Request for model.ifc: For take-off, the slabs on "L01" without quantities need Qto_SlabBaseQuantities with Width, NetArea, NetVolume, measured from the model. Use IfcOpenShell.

First a look at what the model holds.

```python
import ifcopenshell
import ifcopenshell.util.element
import ifcopenshell.util.unit

model = ifcopenshell.open("model.ifc")
print(model.schema)
for unit_type in ("LENGTHUNIT", "AREAUNIT", "VOLUMEUNIT"):
    print(unit_type, ifcopenshell.util.unit.calculate_unit_scale(model, unit_type))
storey = next(s for s in model.by_type("IfcBuildingStorey") if s.Name == "L01")
slabs = [e for e in ifcopenshell.util.element.get_decomposition(storey) if e.is_a("IfcSlab")]
for e in sorted(slabs, key=lambda e: e.id()):
    print(e.id(), e.is_a(), e.Name, list(ifcopenshell.util.element.get_psets(e, qtos_only=True)), sep=" | ")
```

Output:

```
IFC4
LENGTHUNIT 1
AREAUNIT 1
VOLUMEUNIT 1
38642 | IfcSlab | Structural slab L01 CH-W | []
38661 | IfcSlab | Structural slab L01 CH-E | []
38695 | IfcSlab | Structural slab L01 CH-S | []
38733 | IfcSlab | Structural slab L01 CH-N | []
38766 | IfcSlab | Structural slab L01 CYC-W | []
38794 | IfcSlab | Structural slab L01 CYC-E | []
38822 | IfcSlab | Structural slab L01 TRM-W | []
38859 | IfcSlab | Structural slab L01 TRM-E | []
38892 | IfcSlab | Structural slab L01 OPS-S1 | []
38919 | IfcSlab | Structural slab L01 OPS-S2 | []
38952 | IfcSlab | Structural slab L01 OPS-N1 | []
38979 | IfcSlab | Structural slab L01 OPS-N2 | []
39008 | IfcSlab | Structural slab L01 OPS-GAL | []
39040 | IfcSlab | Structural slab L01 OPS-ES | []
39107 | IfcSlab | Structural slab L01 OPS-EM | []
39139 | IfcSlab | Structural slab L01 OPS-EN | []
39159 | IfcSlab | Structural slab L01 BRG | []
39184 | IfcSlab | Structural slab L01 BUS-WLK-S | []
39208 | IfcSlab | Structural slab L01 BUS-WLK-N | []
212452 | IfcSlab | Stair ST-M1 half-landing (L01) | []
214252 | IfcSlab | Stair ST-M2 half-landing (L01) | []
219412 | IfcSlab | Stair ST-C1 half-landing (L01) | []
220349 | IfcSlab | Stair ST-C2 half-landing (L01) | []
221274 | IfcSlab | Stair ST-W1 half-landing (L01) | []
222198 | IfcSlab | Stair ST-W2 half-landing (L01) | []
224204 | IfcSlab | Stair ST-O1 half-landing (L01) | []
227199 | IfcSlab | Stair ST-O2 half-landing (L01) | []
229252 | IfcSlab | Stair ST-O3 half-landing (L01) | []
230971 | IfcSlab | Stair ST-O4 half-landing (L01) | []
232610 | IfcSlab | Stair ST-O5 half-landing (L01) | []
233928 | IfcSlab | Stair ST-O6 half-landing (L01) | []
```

```python
import ifcopenshell
import ifcopenshell.api.pset
import ifcopenshell.geom
import ifcopenshell.util.element
import ifcopenshell.util.shape
import ifcopenshell.util.unit

model = ifcopenshell.open("model.ifc")
unit_scale = ifcopenshell.util.unit.calculate_unit_scale(model)
area_scale = ifcopenshell.util.unit.calculate_unit_scale(model, "AREAUNIT")
volume_scale = ifcopenshell.util.unit.calculate_unit_scale(model, "VOLUMEUNIT")
settings = ifcopenshell.geom.settings()

storey = next(s for s in model.by_type("IfcBuildingStorey") if s.Name == "L01")
slabs = [e for e in ifcopenshell.util.element.get_decomposition(storey) if e.is_a("IfcSlab")]

for e in sorted(slabs, key=lambda e: e.id()):
    if ifcopenshell.util.element.get_psets(e, qtos_only=True, should_inherit=False):
        continue
    # Geometry comes back in metres, in the element's own axes.
    shape = ifcopenshell.geom.create_shape(settings, e)
    values = {
        "Width": ifcopenshell.util.shape.get_z(shape.geometry) / unit_scale,
        "NetArea": ifcopenshell.util.shape.get_footprint_area(shape.geometry) / area_scale,
        "NetVolume": ifcopenshell.util.shape.get_volume(shape.geometry) / volume_scale,
    }
    qto = ifcopenshell.api.pset.add_qto(model, product=e, name="Qto_SlabBaseQuantities")
    ifcopenshell.api.pset.edit_qto(model, qto=qto, properties=values)
    print(e.id(), {k: round(v, 3) for k, v in values.items()})

model.write("model_rev.ifc")
```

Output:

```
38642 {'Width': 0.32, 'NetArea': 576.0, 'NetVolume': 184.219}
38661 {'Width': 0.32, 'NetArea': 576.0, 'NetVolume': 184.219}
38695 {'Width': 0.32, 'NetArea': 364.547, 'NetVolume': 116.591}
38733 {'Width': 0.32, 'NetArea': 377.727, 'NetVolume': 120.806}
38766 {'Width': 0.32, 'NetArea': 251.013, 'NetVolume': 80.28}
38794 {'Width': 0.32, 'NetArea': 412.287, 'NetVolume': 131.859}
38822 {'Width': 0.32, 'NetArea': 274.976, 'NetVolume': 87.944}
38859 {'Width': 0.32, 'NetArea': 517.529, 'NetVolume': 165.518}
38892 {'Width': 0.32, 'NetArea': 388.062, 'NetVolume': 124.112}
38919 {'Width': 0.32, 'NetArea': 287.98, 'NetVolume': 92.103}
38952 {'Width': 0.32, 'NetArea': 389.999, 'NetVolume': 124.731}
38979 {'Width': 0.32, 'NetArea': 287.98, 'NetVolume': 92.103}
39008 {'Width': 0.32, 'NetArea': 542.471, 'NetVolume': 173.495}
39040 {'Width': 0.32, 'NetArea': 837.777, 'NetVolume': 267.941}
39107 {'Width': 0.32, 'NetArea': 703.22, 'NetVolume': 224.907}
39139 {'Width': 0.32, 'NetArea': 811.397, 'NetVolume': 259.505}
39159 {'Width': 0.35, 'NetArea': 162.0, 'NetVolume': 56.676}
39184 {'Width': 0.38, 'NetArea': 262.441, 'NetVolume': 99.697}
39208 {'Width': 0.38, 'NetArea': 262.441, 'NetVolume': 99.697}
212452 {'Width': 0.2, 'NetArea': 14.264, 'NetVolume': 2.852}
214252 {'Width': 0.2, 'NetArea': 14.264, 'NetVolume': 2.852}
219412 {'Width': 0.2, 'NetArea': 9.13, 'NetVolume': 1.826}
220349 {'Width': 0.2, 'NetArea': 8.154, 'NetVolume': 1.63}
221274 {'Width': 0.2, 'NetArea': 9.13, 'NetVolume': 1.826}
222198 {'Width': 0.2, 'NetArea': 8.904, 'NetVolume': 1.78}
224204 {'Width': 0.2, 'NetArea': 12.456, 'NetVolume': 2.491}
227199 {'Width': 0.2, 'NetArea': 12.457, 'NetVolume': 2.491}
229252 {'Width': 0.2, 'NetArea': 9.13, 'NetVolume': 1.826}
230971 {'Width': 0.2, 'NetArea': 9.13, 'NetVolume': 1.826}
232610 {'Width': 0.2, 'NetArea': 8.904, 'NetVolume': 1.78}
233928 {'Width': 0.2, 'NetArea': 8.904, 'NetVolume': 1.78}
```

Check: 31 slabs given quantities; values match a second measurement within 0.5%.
